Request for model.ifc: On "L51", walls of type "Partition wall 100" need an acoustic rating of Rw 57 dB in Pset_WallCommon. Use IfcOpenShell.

First a look at what the model holds.

```python
import ifcopenshell
import ifcopenshell.util.element

model = ifcopenshell.open("model.ifc")
print(model.schema)
storey = next(s for s in model.by_type("IfcBuildingStorey") if s.Name == "L51")
walls = [e for e in ifcopenshell.util.element.get_decomposition(storey) if e.is_a("IfcWall")]
seen = {}
for e in walls:
    element_type = ifcopenshell.util.element.get_type(e)
    key = (element_type.Name if element_type != e and element_type else None, ifcopenshell.util.element.get_pset(e, "Pset_WallCommon", "AcousticRating"))
    seen[key] = seen.get(key, 0) + 1
for (name, value), count in sorted(seen.items(), key=str):
    print(count, "x", name, "|", value)
```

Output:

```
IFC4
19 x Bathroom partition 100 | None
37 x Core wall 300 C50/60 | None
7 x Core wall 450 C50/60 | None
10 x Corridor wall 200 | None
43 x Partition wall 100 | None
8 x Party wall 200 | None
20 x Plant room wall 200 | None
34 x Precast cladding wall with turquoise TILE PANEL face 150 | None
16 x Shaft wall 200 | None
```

```python
import ifcopenshell
import ifcopenshell.api.pset
import ifcopenshell.util.element

model = ifcopenshell.open("model.ifc")

storey = next(s for s in model.by_type("IfcBuildingStorey") if s.Name == "L51")
walls = [e for e in ifcopenshell.util.element.get_decomposition(storey) if e.is_a("IfcWall")]

count = 0
for e in walls:
    element_type = ifcopenshell.util.element.get_type(e)
    if element_type in (None, e) or element_type.Name != "Partition wall 100":
        continue
    found = ifcopenshell.util.element.get_pset(e, "Pset_WallCommon", should_inherit=False)
    if found:
        pset = model.by_id(found["id"])
        if len(ifcopenshell.util.element.get_elements_by_pset(pset)) > 1:
            pset = ifcopenshell.api.pset.unshare_pset(model, products=[e], pset=pset)[0]
    else:
        pset = ifcopenshell.api.pset.add_pset(model, product=e, name="Pset_WallCommon")
    ifcopenshell.api.pset.edit_pset(model, pset=pset, properties={"AcousticRating": "Rw 57 dB"})
    count += 1

print(count, "walls updated")

model.write("model_v2.ifc")
```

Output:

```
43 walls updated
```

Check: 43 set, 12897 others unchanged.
